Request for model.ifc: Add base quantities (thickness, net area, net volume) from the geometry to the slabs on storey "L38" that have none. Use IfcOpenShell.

First a look at what the model holds.

```python
import ifcopenshell
import ifcopenshell.util.element
import ifcopenshell.util.unit

model = ifcopenshell.open("model.ifc")
print(model.schema)
for unit_type in ("LENGTHUNIT", "AREAUNIT", "VOLUMEUNIT"):
    print(unit_type, ifcopenshell.util.unit.calculate_unit_scale(model, unit_type))
storey = next(s for s in model.by_type("IfcBuildingStorey") if s.Name == "L38")
slabs = [e for e in ifcopenshell.util.element.get_decomposition(storey) if e.is_a("IfcSlab")]
for e in sorted(slabs, key=lambda e: e.id()):
    print(e.id(), e.is_a(), e.Name, list(ifcopenshell.util.element.get_psets(e, qtos_only=True)), sep=" | ")
```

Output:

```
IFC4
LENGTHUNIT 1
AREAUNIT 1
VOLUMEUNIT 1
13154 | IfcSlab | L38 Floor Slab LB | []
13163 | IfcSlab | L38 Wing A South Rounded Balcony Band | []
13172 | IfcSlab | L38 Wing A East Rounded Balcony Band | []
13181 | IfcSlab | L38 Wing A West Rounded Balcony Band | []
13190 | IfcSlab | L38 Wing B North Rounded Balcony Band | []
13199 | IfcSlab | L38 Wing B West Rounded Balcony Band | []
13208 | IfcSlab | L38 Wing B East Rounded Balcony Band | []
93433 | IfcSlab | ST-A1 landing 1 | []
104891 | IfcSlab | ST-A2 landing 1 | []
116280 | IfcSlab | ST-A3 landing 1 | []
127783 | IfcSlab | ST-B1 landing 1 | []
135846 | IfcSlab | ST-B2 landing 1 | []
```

```python
import ifcopenshell
import ifcopenshell.api.pset
import ifcopenshell.geom
import ifcopenshell.util.element
import ifcopenshell.util.shape
import ifcopenshell.util.unit

model = ifcopenshell.open("model.ifc")
unit_scale = ifcopenshell.util.unit.calculate_unit_scale(model)
area_scale = ifcopenshell.util.unit.calculate_unit_scale(model, "AREAUNIT")
volume_scale = ifcopenshell.util.unit.calculate_unit_scale(model, "VOLUMEUNIT")
settings = ifcopenshell.geom.settings()

storey = next(s for s in model.by_type("IfcBuildingStorey") if s.Name == "L38")
slabs = [e for e in ifcopenshell.util.element.get_decomposition(storey) if e.is_a("IfcSlab")]

for e in sorted(slabs, key=lambda e: e.id()):
    if ifcopenshell.util.element.get_psets(e, qtos_only=True, should_inherit=False):
        continue
    # Geometry comes back in metres, in the element's own axes.
    shape = ifcopenshell.geom.create_shape(settings, e)
    values = {
        "Width": ifcopenshell.util.shape.get_z(shape.geometry) / unit_scale,
        "NetArea": ifcopenshell.util.shape.get_footprint_area(shape.geometry) / area_scale,
        "NetVolume": ifcopenshell.util.shape.get_volume(shape.geometry) / volume_scale,
    }
    qto = ifcopenshell.api.pset.add_qto(model, product=e, name="Qto_SlabBaseQuantities")
    ifcopenshell.api.pset.edit_qto(model, qto=qto, properties=values)
    print(e.id(), {k: round(v, 3) for k, v in values.items()})

model.write("model_updated.ifc")
```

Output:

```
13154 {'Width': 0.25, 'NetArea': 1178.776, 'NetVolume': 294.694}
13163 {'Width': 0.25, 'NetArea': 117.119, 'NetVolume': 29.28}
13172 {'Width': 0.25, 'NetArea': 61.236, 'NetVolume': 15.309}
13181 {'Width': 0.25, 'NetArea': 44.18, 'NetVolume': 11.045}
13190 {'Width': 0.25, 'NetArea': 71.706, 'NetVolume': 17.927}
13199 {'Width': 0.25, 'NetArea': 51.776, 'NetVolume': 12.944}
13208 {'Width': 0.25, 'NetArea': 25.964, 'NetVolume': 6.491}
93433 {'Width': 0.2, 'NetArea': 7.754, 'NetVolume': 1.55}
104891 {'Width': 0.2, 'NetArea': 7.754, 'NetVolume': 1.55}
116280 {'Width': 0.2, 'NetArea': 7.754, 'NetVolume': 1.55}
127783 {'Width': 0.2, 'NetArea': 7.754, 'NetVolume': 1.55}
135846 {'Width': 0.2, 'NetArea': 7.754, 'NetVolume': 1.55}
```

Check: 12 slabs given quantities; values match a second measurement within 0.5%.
